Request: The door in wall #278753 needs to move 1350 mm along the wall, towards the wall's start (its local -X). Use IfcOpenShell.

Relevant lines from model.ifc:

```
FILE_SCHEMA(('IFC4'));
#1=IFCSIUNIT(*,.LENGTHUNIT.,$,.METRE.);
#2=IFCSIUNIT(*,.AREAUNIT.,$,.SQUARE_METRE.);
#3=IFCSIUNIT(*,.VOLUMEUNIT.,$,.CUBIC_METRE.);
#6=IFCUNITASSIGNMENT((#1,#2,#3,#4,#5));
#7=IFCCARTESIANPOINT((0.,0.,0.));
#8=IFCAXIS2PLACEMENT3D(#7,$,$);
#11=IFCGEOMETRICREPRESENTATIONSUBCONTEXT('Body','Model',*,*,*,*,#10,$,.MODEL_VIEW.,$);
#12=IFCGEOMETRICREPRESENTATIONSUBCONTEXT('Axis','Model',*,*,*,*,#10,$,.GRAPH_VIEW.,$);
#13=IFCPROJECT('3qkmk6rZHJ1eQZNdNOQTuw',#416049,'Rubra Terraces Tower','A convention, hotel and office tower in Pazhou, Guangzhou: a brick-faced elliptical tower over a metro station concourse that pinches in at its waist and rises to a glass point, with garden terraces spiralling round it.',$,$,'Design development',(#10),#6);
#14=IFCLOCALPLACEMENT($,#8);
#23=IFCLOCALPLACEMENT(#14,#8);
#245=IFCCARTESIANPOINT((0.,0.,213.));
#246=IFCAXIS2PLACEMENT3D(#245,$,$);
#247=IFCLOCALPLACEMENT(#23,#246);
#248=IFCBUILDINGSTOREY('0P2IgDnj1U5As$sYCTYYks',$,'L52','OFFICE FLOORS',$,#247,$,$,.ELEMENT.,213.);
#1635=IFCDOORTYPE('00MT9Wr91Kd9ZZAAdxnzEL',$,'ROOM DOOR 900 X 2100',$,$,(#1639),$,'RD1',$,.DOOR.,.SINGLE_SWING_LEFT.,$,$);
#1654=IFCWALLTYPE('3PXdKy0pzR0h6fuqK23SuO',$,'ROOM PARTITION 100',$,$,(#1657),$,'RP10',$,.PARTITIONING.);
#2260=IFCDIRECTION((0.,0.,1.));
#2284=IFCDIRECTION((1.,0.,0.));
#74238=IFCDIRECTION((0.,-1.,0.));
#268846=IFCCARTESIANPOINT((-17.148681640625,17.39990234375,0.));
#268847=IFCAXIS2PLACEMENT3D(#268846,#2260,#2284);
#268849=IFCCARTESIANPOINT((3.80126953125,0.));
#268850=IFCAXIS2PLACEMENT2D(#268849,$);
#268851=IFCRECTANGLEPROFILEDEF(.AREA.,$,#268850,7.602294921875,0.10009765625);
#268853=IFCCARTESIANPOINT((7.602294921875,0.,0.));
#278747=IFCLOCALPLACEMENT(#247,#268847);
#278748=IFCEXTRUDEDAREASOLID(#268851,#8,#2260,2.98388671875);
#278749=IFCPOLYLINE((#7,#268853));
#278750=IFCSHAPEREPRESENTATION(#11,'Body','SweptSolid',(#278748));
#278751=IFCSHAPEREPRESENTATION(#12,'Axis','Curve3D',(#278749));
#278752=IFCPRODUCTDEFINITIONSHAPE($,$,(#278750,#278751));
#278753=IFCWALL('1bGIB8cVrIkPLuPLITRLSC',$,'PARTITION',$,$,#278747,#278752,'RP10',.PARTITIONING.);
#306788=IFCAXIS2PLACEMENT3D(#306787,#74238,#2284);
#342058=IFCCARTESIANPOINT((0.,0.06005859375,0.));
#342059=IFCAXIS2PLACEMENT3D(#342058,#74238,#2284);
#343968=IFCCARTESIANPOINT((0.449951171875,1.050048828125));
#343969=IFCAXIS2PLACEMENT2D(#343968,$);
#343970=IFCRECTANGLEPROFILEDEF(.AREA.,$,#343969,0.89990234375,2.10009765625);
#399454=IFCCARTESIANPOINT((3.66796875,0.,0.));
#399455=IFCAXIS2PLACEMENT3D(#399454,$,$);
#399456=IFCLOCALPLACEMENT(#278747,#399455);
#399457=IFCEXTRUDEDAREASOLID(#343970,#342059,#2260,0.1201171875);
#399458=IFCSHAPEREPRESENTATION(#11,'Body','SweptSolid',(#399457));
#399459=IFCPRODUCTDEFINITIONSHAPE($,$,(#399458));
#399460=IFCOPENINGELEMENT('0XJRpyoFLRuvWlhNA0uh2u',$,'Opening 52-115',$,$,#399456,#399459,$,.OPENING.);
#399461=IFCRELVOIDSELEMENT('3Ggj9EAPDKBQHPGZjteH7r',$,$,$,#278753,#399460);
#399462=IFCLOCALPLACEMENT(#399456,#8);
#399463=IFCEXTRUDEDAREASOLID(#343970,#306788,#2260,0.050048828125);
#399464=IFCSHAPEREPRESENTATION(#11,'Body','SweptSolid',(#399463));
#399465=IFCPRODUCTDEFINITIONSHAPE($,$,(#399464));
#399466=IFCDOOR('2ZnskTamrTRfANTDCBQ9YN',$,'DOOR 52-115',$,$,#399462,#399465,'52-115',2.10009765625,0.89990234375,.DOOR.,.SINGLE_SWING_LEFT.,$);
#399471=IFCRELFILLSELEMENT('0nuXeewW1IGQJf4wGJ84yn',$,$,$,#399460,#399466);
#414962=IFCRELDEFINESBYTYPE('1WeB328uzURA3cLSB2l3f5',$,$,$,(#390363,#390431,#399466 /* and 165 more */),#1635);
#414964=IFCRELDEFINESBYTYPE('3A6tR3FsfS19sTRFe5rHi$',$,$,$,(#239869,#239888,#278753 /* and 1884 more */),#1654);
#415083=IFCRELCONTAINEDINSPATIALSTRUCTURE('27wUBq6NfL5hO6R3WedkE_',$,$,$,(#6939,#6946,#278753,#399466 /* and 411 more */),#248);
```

```python
import ifcopenshell
import ifcopenshell.api.geometry
import ifcopenshell.util.placement
import ifcopenshell.util.unit

model = ifcopenshell.open("model.ifc")
unit_scale = ifcopenshell.util.unit.calculate_unit_scale(model)

door = model.by_guid("2ZnskTamrTRfANTDCBQ9YN")
opening = door.FillsVoids[0].RelatingOpeningElement
wall = opening.VoidsElements[0].RelatingBuildingElement

wall_matrix = ifcopenshell.util.placement.get_local_placement(wall.ObjectPlacement)
shift = wall_matrix[:3, 0] * -1.35 / unit_scale
before = ifcopenshell.util.placement.get_local_placement(door.ObjectPlacement)[:3, 3].copy()

# The door is placed relative to its opening, so it follows when the opening moves.
matrix = ifcopenshell.util.placement.get_local_placement(opening.ObjectPlacement)
matrix[:3, 3] += shift
ifcopenshell.api.geometry.edit_object_placement(
    model, product=opening, matrix=matrix, is_si=False, should_transform_children=True
)

after = ifcopenshell.util.placement.get_local_placement(door.ObjectPlacement)[:3, 3]
print("door moved by", (after - before).round(3) + 0.0)

model.write("model_edited.ifc")
```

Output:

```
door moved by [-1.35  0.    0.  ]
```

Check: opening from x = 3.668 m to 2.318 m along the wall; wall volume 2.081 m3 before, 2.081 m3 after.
